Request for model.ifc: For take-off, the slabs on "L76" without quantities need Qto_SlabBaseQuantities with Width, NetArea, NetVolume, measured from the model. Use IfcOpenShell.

First a look at what the model holds.

```python
import ifcopenshell
import ifcopenshell.util.element
import ifcopenshell.util.unit

model = ifcopenshell.open("model.ifc")
print(model.schema)
for unit_type in ("LENGTHUNIT", "AREAUNIT", "VOLUMEUNIT"):
    print(unit_type, ifcopenshell.util.unit.calculate_unit_scale(model, unit_type))
storey = next(s for s in model.by_type("IfcBuildingStorey") if s.Name == "L76")
slabs = [e for e in ifcopenshell.util.element.get_decomposition(storey) if e.is_a("IfcSlab")]
for e in sorted(slabs, key=lambda e: e.id()):
    print(e.id(), e.is_a(), e.Name, list(ifcopenshell.util.element.get_psets(e, qtos_only=True)), sep=" | ")
```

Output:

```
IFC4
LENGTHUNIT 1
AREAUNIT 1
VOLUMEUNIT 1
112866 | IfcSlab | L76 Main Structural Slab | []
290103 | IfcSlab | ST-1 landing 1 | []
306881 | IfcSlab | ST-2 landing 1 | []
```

```python
import ifcopenshell
import ifcopenshell.api.pset
import ifcopenshell.geom
import ifcopenshell.util.element
import ifcopenshell.util.shape
import ifcopenshell.util.unit

model = ifcopenshell.open("model.ifc")
unit_scale = ifcopenshell.util.unit.calculate_unit_scale(model)
area_scale = ifcopenshell.util.unit.calculate_unit_scale(model, "AREAUNIT")
volume_scale = ifcopenshell.util.unit.calculate_unit_scale(model, "VOLUMEUNIT")
settings = ifcopenshell.geom.settings()

storey = next(s for s in model.by_type("IfcBuildingStorey") if s.Name == "L76")
slabs = [e for e in ifcopenshell.util.element.get_decomposition(storey) if e.is_a("IfcSlab")]

for e in sorted(slabs, key=lambda e: e.id()):
    if ifcopenshell.util.element.get_psets(e, qtos_only=True, should_inherit=False):
        continue
    # Geometry comes back in metres, in the element's own axes.
    shape = ifcopenshell.geom.create_shape(settings, e)
    values = {
        "Width": ifcopenshell.util.shape.get_z(shape.geometry) / unit_scale,
        "NetArea": ifcopenshell.util.shape.get_footprint_area(shape.geometry) / area_scale,
        "NetVolume": ifcopenshell.util.shape.get_volume(shape.geometry) / volume_scale,
    }
    qto = ifcopenshell.api.pset.add_qto(model, product=e, name="Qto_SlabBaseQuantities")
    ifcopenshell.api.pset.edit_qto(model, qto=qto, properties=values)
    print(e.id(), {k: round(v, 3) for k, v in values.items()})

model.write("model_edited.ifc")
```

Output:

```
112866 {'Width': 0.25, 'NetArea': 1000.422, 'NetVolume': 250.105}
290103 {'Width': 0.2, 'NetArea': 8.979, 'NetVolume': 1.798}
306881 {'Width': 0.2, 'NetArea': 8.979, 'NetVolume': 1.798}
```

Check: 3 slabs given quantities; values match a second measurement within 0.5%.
